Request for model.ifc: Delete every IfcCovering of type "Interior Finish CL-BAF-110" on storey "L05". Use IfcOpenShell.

First a look at what the model holds.

```python
import ifcopenshell
import ifcopenshell.util.element

model = ifcopenshell.open("model.ifc")
print(model.schema)
storey = next(s for s in model.by_type("IfcBuildingStorey") if s.Name == "L05")
coverings = [e for e in ifcopenshell.util.element.get_decomposition(storey) if e.is_a("IfcCovering")]
seen = {}
for e in coverings:
    element_type = ifcopenshell.util.element.get_type(e)
    name = element_type.Name if element_type not in (None, e) else None
    seen[name] = seen.get(name, 0) + 1
for name, count in sorted(seen.items(), key=str):
    print(count, "x", name)
```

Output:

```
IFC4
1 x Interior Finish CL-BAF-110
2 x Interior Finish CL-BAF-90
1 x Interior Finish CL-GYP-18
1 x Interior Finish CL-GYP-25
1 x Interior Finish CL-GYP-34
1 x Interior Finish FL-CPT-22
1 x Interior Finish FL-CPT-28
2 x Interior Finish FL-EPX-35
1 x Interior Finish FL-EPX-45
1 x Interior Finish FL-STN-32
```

```python
import ifcopenshell
import ifcopenshell.api.root
import ifcopenshell.util.element

model = ifcopenshell.open("model.ifc")

storey = next(s for s in model.by_type("IfcBuildingStorey") if s.Name == "L05")
coverings = [e for e in ifcopenshell.util.element.get_decomposition(storey) if e.is_a("IfcCovering")]
targets = [e for e in coverings if (t := ifcopenshell.util.element.get_type(e)) not in (None, e) and t.Name == "Interior Finish CL-BAF-110"]

for e in targets:
    ifcopenshell.api.root.remove_product(model, product=e)
print(len(targets), "removed")

model.write("model_rev.ifc")
```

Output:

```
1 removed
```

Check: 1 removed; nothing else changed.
